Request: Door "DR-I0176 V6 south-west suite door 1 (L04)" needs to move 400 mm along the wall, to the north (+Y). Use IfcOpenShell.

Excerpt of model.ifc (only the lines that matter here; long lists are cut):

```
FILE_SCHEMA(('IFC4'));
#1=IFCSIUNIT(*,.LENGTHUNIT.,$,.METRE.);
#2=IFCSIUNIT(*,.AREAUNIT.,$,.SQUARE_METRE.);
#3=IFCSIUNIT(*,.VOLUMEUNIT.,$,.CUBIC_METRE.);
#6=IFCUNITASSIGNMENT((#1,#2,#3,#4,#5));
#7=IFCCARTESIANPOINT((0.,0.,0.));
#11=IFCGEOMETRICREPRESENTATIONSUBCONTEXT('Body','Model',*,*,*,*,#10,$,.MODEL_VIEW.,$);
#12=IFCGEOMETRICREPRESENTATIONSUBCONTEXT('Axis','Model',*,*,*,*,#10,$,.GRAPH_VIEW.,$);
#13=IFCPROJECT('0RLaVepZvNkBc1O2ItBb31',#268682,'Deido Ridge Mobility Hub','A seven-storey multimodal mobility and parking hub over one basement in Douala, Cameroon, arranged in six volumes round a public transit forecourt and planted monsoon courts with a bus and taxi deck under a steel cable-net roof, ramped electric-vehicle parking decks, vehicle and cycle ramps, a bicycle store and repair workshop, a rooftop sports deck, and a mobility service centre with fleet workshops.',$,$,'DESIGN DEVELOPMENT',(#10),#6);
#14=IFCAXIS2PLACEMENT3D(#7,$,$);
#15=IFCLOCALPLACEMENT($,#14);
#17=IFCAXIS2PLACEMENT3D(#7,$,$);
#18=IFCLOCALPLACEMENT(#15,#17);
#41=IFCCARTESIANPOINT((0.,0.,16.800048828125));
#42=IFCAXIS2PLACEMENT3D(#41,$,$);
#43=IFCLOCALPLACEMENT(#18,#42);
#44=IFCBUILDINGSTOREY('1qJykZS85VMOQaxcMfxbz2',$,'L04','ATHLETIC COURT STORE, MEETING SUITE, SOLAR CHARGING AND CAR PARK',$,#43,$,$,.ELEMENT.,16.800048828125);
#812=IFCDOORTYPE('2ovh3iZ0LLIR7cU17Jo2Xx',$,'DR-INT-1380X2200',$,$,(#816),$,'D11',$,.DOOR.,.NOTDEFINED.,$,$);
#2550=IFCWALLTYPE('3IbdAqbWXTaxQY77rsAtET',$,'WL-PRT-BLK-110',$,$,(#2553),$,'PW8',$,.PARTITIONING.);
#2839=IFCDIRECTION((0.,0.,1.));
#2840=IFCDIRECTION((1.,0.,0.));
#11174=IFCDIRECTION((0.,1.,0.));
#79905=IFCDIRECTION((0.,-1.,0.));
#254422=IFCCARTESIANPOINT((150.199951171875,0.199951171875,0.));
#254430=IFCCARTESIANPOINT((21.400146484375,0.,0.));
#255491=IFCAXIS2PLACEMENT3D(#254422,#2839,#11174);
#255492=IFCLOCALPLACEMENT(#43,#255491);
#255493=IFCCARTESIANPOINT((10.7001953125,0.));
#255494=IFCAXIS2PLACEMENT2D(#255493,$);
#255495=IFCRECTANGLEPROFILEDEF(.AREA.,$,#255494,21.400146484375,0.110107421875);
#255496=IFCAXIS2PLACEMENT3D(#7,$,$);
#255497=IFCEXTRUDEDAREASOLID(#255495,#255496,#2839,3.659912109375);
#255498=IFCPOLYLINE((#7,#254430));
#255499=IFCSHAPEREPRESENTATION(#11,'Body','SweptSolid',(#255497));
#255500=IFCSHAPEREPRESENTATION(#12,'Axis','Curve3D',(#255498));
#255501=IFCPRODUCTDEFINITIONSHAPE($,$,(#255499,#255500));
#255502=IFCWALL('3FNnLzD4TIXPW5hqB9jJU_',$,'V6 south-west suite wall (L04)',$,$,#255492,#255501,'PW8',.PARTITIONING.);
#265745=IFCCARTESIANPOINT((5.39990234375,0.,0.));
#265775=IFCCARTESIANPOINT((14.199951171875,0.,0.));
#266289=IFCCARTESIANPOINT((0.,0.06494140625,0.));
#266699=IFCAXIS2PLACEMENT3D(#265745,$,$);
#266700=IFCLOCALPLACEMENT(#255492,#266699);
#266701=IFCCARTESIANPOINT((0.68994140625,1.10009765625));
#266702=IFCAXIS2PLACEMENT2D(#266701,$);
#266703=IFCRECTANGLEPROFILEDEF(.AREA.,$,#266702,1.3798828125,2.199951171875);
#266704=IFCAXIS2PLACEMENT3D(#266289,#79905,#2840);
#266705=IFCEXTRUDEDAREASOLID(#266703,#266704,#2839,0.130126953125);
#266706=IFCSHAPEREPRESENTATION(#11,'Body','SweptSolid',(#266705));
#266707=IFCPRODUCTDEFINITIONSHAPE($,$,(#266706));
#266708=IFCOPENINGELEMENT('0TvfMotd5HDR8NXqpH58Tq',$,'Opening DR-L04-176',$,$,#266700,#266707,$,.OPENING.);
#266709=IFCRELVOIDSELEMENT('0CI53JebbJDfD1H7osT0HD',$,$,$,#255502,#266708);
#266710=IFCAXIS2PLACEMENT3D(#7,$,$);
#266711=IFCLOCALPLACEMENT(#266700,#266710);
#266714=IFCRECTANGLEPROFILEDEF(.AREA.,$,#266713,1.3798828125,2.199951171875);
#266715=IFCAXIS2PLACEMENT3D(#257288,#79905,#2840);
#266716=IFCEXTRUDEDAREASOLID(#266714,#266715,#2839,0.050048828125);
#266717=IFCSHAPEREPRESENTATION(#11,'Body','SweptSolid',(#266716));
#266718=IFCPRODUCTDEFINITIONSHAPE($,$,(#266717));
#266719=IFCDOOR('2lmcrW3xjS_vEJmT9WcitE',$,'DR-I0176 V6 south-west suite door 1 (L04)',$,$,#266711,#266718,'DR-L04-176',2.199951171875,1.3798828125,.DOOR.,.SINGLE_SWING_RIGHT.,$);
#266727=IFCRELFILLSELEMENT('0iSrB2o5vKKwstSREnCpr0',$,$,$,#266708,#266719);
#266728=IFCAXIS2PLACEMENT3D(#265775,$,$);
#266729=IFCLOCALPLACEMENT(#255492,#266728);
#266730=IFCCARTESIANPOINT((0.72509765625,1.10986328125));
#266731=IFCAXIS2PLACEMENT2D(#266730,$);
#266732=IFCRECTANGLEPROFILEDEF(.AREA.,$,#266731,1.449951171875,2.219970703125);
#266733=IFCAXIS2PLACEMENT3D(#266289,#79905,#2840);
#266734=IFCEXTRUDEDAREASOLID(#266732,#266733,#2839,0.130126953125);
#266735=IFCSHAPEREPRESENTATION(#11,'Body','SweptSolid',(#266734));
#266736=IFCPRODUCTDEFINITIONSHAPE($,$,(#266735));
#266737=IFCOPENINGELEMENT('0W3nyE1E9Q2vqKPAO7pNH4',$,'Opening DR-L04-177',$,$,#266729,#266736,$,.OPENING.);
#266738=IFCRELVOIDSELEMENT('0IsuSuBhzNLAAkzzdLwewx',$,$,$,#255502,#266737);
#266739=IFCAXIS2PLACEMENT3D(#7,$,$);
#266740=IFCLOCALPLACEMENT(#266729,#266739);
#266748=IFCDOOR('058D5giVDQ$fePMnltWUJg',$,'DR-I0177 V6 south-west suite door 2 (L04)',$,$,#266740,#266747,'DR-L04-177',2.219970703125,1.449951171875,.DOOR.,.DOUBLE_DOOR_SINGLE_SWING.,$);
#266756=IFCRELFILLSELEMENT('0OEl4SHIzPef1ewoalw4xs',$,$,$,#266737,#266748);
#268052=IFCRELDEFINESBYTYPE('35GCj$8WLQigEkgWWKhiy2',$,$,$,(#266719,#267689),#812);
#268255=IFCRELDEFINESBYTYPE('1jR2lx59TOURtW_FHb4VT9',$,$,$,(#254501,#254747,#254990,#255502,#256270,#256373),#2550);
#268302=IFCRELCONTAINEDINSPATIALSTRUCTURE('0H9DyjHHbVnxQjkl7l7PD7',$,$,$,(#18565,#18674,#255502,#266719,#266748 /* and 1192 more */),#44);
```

```python
import ifcopenshell
import ifcopenshell.api.geometry
import ifcopenshell.util.placement
import ifcopenshell.util.unit

model = ifcopenshell.open("model.ifc")
unit_scale = ifcopenshell.util.unit.calculate_unit_scale(model)

door = model.by_guid("2lmcrW3xjS_vEJmT9WcitE")
opening = door.FillsVoids[0].RelatingOpeningElement
wall = opening.VoidsElements[0].RelatingBuildingElement

wall_matrix = ifcopenshell.util.placement.get_local_placement(wall.ObjectPlacement)
shift = wall_matrix[:3, 0] * 0.4 / unit_scale
before = ifcopenshell.util.placement.get_local_placement(door.ObjectPlacement)[:3, 3].copy()

# The door is placed relative to its opening, so it follows when the opening moves.
matrix = ifcopenshell.util.placement.get_local_placement(opening.ObjectPlacement)
matrix[:3, 3] += shift
ifcopenshell.api.geometry.edit_object_placement(
    model, product=opening, matrix=matrix, is_si=False, should_transform_children=True
)

after = ifcopenshell.util.placement.get_local_placement(door.ObjectPlacement)[:3, 3]
print("door moved by", (after - before).round(3) + 0.0)

model.write("model_rev.ifc")
```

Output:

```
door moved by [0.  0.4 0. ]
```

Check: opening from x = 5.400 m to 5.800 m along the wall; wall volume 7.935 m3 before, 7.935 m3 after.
